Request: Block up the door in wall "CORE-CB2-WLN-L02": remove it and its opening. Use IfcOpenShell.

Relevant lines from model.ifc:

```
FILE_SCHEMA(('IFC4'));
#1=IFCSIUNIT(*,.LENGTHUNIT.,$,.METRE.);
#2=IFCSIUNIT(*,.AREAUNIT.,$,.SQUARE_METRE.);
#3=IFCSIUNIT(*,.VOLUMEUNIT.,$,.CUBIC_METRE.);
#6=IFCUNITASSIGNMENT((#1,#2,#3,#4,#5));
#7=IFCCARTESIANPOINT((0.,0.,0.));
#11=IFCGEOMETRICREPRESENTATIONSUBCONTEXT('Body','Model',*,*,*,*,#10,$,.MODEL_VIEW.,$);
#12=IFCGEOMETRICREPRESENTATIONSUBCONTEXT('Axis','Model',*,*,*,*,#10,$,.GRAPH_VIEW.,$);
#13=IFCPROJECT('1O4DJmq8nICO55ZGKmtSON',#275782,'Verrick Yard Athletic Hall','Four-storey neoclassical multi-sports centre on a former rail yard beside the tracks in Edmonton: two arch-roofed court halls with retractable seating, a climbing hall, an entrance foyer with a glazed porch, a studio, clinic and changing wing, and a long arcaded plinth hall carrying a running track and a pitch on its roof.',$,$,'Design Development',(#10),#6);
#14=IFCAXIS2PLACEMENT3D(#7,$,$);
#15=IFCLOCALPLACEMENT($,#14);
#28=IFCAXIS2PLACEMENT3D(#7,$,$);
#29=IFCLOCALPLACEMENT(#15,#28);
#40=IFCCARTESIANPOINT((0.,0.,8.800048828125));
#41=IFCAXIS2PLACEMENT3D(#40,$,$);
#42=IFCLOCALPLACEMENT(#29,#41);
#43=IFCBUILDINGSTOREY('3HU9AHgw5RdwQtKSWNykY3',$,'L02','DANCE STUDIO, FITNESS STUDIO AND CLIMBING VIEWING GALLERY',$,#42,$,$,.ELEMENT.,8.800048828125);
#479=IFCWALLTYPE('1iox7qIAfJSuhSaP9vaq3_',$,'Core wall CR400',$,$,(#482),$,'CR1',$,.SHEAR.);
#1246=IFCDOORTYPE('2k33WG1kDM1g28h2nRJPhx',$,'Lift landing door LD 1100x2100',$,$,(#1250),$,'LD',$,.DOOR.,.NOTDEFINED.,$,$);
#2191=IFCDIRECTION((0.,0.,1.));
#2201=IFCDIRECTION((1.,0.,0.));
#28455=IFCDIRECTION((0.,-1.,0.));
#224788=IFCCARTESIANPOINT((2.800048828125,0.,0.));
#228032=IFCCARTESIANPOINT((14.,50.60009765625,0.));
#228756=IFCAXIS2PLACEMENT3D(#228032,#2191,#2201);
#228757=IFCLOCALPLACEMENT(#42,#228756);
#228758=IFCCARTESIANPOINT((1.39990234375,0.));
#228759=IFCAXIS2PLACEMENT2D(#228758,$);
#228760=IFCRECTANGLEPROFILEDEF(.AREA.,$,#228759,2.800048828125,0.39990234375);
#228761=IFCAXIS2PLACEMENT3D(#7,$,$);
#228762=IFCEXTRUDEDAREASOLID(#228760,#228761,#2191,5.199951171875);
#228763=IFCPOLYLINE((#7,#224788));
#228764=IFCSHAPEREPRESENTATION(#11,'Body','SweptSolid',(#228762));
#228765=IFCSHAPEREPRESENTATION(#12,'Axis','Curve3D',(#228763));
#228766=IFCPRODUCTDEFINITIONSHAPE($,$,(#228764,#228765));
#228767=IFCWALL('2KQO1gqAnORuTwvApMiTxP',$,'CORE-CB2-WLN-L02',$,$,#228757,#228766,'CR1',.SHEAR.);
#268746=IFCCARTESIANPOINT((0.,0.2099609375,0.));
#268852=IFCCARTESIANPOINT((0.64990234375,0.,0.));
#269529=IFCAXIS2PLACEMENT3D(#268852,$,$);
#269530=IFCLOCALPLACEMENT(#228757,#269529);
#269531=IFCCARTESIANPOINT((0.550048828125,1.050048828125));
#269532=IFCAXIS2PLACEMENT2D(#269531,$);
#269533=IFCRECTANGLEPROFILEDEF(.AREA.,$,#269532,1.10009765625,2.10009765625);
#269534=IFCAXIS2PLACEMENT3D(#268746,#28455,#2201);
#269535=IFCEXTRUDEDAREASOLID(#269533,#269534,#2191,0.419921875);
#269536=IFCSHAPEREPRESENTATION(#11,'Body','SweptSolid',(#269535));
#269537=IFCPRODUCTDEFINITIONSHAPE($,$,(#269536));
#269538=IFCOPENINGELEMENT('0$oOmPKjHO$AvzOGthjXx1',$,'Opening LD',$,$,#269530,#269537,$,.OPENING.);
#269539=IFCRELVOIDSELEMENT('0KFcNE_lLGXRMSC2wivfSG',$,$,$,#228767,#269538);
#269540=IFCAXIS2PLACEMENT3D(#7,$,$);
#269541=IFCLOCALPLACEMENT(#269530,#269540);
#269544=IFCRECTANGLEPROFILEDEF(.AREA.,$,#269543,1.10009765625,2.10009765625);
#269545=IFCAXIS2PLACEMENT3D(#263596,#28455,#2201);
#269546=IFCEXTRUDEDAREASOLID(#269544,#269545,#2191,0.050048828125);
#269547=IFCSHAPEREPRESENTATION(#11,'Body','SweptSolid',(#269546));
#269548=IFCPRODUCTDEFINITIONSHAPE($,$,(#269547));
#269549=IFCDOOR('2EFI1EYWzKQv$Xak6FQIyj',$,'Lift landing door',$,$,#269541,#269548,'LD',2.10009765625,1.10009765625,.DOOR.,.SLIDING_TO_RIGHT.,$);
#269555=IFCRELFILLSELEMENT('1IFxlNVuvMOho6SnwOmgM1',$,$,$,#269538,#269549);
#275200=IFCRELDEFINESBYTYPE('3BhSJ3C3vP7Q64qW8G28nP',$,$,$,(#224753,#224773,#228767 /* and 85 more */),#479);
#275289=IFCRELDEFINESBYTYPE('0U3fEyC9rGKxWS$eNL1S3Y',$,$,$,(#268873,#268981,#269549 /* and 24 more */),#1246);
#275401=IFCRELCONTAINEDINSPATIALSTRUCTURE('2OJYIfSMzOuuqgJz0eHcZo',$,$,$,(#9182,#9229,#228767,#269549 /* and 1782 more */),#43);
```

```python
import ifcopenshell
import ifcopenshell.api.feature
import ifcopenshell.api.root
import ifcopenshell.geom
import ifcopenshell.util.shape

model = ifcopenshell.open("model.ifc")
settings = ifcopenshell.geom.settings()


def volume(element):
    """Net volume in cubic metres, openings subtracted."""
    shape = ifcopenshell.geom.create_shape(settings, element)
    return ifcopenshell.util.shape.get_volume(shape.geometry)


door = model.by_guid("2EFI1EYWzKQv$Xak6FQIyj")
opening = door.FillsVoids[0].RelatingOpeningElement
wall = opening.VoidsElements[0].RelatingBuildingElement
before = volume(wall)

ifcopenshell.api.root.remove_product(model, product=door)
ifcopenshell.api.feature.remove_feature(model, feature=opening)

after = volume(wall)

print(f"wall volume {before:.3f} -> {after:.3f} m3")

model.write("model_edited.ifc")
```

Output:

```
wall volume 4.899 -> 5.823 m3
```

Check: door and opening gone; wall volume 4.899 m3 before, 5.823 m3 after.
